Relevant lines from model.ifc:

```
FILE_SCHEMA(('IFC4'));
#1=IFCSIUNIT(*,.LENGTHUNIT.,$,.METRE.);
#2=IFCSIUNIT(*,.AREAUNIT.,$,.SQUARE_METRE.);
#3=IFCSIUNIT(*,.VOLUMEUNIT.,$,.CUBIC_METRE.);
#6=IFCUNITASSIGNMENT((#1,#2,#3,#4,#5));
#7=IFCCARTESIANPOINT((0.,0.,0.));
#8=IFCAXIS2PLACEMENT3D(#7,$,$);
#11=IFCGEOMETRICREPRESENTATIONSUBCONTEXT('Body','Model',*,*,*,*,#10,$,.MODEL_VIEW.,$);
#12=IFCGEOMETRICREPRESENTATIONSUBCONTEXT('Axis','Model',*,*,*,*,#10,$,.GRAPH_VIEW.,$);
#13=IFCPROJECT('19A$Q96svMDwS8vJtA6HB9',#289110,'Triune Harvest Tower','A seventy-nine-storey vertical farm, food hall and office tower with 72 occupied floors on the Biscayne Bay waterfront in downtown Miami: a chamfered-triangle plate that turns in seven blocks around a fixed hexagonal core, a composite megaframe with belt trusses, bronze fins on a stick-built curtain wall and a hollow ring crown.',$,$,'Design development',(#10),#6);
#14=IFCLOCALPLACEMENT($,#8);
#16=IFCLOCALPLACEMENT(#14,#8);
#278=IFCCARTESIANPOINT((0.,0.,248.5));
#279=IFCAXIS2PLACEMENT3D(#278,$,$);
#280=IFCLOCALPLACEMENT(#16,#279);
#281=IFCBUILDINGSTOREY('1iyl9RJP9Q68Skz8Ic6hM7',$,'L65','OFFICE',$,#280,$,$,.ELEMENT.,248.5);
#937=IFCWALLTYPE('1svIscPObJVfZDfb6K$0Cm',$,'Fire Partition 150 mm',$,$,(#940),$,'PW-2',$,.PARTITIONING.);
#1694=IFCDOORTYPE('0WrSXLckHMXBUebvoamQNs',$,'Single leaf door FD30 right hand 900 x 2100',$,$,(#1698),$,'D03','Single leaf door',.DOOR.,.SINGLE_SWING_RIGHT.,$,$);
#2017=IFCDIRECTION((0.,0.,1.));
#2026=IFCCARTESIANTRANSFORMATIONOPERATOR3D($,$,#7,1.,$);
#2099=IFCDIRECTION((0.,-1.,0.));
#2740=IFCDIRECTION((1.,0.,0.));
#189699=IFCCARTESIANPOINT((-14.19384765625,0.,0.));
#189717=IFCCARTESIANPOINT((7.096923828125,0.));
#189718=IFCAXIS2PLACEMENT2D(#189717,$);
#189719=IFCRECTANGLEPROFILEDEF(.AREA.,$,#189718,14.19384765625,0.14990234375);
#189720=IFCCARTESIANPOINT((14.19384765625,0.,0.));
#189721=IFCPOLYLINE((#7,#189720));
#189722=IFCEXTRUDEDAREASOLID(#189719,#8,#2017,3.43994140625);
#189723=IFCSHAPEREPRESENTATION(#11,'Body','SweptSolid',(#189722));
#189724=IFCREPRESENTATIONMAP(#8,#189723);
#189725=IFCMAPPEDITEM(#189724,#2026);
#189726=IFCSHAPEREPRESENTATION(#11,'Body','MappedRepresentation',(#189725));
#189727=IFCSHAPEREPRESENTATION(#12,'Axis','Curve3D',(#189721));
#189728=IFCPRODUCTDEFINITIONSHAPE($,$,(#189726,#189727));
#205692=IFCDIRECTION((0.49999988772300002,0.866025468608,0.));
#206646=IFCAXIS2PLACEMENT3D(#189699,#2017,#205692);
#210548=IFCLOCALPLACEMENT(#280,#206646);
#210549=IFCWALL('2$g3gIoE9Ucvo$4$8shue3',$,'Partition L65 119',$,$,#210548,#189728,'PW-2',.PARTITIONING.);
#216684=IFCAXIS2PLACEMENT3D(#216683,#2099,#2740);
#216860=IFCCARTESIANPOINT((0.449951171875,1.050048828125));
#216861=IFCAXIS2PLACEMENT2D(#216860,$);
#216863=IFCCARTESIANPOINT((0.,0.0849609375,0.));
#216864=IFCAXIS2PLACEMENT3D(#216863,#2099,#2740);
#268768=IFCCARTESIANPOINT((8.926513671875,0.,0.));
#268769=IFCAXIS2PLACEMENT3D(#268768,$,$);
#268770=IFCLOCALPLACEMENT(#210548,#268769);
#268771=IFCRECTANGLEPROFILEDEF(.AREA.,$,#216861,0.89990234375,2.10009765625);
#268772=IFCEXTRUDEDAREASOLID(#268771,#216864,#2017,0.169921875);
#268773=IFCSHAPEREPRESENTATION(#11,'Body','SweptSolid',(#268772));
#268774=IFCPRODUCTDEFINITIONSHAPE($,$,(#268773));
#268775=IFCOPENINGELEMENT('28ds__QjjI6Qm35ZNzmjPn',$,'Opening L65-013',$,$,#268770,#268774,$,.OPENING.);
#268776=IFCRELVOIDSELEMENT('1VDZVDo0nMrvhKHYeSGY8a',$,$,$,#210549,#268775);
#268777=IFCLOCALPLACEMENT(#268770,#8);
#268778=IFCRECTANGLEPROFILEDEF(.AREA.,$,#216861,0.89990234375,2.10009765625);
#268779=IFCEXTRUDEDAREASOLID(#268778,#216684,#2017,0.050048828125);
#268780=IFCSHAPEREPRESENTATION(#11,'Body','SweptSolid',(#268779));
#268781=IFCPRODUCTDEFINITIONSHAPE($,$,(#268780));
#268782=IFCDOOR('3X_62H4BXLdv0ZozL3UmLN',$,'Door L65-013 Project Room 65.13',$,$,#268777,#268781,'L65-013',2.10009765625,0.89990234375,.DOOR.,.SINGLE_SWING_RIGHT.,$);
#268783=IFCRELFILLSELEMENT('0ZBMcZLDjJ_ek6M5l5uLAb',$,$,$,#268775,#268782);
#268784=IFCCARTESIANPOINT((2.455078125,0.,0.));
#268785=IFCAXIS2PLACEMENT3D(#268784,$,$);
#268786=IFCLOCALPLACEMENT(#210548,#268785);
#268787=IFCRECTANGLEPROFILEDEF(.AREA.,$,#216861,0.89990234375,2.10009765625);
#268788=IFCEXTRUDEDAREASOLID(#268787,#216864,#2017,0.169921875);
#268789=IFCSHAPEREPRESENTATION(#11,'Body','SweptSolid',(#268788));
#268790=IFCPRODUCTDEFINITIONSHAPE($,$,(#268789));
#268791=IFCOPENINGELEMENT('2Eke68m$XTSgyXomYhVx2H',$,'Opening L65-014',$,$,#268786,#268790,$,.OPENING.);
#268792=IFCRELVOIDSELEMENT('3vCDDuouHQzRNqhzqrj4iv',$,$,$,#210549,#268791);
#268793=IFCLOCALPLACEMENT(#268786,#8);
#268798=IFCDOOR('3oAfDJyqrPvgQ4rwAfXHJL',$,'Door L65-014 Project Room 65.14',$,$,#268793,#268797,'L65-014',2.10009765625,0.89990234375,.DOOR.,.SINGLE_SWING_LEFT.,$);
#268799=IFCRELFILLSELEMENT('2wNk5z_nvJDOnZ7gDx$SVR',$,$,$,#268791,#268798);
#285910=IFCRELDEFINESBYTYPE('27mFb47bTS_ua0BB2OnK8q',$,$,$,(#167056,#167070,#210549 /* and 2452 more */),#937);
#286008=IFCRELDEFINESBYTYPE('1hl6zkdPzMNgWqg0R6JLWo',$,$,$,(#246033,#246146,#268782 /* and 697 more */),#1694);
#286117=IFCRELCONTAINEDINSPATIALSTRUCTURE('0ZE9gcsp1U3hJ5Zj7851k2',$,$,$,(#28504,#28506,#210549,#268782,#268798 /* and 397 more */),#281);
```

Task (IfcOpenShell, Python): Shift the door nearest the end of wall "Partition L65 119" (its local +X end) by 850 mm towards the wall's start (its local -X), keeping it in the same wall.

```python
import ifcopenshell
import ifcopenshell.api.geometry
import ifcopenshell.util.placement
import ifcopenshell.util.unit

model = ifcopenshell.open("model.ifc")
unit_scale = ifcopenshell.util.unit.calculate_unit_scale(model)

door = model.by_guid("3X_62H4BXLdv0ZozL3UmLN")
opening = door.FillsVoids[0].RelatingOpeningElement
wall = opening.VoidsElements[0].RelatingBuildingElement

wall_matrix = ifcopenshell.util.placement.get_local_placement(wall.ObjectPlacement)
shift = wall_matrix[:3, 0] * -0.85 / unit_scale
before = ifcopenshell.util.placement.get_local_placement(door.ObjectPlacement)[:3, 3].copy()

# The door is placed relative to its opening, so it follows when the opening moves.
matrix = ifcopenshell.util.placement.get_local_placement(opening.ObjectPlacement)
matrix[:3, 3] += shift
ifcopenshell.api.geometry.edit_object_placement(
    model, product=opening, matrix=matrix, is_si=False, should_transform_children=True
)

after = ifcopenshell.util.placement.get_local_placement(door.ObjectPlacement)[:3, 3]
print("door moved by", (after - before).round(3) + 0.0)

model.write("model-out.ifc")
```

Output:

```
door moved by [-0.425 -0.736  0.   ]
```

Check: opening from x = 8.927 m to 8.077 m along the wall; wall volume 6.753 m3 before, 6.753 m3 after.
